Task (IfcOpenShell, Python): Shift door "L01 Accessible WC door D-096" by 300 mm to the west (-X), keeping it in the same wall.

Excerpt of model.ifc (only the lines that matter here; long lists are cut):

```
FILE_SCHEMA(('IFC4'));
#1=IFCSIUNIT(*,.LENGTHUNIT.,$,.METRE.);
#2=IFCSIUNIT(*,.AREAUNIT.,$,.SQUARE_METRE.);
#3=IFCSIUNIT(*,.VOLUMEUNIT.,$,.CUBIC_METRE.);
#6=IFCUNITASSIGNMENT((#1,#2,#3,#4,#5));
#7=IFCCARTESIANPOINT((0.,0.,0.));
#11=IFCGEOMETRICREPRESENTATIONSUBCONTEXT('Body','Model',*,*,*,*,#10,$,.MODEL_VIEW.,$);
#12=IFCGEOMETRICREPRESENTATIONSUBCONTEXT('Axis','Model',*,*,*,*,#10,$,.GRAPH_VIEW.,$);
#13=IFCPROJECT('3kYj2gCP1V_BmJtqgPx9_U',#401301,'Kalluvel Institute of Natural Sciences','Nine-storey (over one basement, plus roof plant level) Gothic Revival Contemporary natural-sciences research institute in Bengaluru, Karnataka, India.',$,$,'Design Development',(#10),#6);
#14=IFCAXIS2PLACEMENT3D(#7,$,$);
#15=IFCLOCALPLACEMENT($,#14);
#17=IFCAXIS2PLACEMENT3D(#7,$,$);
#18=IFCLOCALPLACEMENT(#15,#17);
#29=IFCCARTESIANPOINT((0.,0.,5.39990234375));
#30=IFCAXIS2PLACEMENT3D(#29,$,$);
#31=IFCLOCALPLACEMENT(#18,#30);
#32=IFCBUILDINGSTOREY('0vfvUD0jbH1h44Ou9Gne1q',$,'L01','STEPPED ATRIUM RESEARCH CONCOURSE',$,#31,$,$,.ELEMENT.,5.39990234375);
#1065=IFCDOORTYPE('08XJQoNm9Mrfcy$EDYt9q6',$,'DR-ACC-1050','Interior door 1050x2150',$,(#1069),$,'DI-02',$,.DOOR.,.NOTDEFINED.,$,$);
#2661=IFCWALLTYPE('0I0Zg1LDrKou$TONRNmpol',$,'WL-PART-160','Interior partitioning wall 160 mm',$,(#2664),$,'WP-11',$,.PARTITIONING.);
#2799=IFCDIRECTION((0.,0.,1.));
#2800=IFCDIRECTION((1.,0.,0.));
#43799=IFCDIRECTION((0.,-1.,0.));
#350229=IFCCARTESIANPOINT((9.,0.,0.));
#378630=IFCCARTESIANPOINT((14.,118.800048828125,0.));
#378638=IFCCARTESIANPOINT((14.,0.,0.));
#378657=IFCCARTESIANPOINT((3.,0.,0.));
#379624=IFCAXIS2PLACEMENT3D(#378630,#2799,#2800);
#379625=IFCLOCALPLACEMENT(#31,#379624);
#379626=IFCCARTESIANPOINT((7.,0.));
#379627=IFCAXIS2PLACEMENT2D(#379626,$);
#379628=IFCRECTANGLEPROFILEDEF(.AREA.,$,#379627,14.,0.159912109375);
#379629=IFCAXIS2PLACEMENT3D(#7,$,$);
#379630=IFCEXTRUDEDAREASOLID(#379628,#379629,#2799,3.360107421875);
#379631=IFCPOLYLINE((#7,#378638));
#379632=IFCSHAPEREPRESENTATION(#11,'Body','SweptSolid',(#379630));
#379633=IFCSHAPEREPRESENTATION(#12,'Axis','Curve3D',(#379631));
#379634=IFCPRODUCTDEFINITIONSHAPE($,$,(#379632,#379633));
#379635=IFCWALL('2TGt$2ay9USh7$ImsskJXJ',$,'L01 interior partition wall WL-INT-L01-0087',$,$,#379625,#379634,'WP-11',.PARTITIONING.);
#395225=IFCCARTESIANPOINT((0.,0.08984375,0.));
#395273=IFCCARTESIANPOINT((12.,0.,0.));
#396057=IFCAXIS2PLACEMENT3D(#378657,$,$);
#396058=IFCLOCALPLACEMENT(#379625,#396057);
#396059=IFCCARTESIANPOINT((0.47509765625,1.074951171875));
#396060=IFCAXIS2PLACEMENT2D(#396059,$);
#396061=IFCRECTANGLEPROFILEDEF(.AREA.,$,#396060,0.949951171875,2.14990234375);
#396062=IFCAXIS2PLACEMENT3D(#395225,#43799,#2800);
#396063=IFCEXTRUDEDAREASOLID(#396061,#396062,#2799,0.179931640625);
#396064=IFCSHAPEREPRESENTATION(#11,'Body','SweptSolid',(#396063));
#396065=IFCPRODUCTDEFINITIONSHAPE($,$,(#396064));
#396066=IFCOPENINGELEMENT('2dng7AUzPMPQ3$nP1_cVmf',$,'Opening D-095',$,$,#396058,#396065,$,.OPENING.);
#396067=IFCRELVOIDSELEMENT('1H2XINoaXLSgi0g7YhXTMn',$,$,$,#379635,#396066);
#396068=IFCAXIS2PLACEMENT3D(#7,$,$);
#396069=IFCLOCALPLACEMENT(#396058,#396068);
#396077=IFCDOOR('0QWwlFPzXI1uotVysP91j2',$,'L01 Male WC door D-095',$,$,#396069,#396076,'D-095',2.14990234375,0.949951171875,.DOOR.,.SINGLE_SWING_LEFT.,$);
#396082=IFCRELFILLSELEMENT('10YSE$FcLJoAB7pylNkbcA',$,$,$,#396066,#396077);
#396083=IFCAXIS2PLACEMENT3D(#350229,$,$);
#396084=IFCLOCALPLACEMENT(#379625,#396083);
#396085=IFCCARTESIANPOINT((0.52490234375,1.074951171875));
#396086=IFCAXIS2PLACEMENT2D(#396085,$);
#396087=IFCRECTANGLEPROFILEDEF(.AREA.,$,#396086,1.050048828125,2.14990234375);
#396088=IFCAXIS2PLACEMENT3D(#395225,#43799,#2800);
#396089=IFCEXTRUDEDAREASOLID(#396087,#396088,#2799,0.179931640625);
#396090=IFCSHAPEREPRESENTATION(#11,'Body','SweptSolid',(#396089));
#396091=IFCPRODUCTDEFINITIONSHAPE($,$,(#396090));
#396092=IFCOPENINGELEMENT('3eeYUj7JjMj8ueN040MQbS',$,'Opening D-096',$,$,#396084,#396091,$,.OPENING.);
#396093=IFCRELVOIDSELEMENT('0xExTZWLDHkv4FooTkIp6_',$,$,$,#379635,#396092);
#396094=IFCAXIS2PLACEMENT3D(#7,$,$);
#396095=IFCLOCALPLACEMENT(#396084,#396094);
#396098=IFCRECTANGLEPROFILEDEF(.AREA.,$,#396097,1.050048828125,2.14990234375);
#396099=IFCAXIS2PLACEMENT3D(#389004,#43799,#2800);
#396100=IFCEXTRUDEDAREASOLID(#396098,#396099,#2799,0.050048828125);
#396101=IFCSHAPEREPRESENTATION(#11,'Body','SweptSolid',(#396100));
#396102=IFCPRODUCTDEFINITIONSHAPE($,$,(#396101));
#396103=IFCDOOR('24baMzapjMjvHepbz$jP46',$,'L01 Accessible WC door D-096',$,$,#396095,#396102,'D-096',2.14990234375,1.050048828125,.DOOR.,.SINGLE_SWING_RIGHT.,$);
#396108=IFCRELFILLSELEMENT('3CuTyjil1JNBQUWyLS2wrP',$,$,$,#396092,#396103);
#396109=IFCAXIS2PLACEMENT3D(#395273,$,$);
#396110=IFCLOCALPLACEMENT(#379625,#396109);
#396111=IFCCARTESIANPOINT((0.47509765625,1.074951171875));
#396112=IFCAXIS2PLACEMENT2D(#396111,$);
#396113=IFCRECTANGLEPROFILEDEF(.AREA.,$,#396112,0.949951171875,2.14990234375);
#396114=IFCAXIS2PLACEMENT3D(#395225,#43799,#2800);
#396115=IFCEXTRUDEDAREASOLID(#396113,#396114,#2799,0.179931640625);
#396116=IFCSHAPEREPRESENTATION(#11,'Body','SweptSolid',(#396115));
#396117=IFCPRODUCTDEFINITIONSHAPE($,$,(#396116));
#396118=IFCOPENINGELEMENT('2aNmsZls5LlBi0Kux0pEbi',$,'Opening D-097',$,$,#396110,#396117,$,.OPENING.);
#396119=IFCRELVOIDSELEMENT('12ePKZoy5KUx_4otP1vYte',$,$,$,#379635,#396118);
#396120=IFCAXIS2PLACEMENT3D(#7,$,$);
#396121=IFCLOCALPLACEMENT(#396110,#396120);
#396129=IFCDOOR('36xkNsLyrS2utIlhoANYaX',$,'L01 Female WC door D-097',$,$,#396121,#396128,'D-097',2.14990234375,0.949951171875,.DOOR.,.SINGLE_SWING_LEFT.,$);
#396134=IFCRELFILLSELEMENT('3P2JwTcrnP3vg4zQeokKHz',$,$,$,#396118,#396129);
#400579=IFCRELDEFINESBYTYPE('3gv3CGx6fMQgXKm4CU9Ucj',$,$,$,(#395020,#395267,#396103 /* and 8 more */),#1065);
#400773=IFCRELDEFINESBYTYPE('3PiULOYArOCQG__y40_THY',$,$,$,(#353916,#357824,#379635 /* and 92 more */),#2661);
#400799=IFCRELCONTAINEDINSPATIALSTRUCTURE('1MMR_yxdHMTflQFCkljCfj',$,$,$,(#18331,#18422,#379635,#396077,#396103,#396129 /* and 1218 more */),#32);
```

```python
import ifcopenshell
import ifcopenshell.api.geometry
import ifcopenshell.util.placement
import ifcopenshell.util.unit

model = ifcopenshell.open("model.ifc")
unit_scale = ifcopenshell.util.unit.calculate_unit_scale(model)

door = model.by_guid("24baMzapjMjvHepbz$jP46")
opening = door.FillsVoids[0].RelatingOpeningElement
wall = opening.VoidsElements[0].RelatingBuildingElement

wall_matrix = ifcopenshell.util.placement.get_local_placement(wall.ObjectPlacement)
shift = wall_matrix[:3, 0] * -0.3 / unit_scale
before = ifcopenshell.util.placement.get_local_placement(door.ObjectPlacement)[:3, 3].copy()

# The door is placed relative to its opening, so it follows when the opening moves.
matrix = ifcopenshell.util.placement.get_local_placement(opening.ObjectPlacement)
matrix[:3, 3] += shift
ifcopenshell.api.geometry.edit_object_placement(
    model, product=opening, matrix=matrix, is_si=False, should_transform_children=True
)

after = ifcopenshell.util.placement.get_local_placement(door.ObjectPlacement)[:3, 3]
print("door moved by", (after - before).round(3) + 0.0)

model.write("model_v2.ifc")
```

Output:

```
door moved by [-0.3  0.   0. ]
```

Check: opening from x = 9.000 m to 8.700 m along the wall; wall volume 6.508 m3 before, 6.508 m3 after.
